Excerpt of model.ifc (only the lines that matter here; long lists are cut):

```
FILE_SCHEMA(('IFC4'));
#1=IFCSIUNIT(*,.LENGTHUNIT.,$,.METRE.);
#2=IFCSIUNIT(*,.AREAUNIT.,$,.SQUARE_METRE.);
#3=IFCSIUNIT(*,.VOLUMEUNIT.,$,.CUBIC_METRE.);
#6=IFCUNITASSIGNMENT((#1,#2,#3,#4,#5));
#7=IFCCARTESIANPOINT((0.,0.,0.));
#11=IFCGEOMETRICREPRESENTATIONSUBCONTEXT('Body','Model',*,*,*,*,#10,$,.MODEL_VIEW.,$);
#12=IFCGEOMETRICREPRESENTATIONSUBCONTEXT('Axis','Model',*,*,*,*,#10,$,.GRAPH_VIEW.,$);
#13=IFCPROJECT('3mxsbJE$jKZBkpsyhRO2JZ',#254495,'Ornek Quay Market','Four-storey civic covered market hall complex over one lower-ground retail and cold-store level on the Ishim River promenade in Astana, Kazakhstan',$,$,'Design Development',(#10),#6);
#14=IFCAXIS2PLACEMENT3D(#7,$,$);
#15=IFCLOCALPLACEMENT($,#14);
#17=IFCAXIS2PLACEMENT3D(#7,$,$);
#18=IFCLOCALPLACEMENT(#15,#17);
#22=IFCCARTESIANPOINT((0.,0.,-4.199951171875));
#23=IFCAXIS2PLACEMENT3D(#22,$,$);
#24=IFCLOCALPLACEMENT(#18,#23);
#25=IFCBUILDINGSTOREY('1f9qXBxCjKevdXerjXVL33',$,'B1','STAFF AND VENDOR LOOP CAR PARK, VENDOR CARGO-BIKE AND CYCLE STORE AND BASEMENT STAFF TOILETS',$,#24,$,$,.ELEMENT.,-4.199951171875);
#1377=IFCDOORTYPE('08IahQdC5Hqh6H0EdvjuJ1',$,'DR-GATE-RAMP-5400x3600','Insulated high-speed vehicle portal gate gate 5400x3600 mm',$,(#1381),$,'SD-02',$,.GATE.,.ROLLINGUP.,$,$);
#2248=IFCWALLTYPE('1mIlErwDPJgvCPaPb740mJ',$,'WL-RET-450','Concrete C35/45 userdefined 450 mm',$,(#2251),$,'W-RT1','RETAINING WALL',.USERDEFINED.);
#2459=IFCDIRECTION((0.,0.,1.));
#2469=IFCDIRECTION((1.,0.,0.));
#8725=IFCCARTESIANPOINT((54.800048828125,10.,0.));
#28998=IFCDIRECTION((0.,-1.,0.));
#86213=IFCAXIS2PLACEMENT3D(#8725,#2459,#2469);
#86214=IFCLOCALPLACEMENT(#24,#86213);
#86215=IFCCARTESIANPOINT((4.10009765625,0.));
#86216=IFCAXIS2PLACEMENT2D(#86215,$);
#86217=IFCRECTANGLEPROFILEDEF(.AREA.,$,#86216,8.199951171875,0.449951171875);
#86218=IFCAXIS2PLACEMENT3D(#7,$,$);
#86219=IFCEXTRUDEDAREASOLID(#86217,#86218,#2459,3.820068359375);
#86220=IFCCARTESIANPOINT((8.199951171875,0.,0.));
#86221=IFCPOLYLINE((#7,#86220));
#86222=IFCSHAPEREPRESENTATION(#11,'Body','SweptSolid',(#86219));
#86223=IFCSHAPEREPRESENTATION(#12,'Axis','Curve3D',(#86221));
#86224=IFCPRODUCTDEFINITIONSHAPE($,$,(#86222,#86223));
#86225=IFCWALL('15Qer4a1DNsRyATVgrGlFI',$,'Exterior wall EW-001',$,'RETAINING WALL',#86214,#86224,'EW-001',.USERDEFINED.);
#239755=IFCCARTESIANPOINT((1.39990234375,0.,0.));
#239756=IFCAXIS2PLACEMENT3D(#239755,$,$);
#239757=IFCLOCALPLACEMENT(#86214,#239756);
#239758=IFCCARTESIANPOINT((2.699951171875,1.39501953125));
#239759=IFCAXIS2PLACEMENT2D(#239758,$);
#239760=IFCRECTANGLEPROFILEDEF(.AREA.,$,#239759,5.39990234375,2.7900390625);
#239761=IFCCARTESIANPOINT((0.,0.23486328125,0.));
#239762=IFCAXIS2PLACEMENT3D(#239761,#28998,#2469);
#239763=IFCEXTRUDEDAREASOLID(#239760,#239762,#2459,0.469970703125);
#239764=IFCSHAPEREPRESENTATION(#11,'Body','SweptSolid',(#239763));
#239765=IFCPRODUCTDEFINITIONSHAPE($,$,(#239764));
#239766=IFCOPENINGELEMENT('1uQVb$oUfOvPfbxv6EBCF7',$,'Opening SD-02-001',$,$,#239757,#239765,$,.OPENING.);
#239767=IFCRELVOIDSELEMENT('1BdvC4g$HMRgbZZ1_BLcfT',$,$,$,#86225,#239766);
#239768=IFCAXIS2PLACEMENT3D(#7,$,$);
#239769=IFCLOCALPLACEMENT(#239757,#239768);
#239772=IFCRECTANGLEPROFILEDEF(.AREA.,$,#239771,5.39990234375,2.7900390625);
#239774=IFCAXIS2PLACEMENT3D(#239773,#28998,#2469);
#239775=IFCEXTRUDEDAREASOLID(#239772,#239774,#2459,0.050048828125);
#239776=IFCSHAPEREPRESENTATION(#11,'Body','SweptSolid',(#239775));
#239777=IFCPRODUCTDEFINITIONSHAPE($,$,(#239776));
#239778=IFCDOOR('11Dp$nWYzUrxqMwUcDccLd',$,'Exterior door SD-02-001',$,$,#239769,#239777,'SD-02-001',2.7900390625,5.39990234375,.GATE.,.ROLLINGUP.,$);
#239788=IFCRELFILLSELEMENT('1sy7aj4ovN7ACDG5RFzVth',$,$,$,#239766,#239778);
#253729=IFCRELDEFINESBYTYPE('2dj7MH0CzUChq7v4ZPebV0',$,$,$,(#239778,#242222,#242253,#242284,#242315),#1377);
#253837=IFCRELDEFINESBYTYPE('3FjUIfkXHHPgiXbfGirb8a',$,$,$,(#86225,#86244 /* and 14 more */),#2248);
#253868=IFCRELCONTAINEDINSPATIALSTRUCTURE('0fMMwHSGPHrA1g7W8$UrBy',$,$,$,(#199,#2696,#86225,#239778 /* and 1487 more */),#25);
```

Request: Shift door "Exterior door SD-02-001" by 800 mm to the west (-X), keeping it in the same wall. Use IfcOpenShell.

```python
import ifcopenshell
import ifcopenshell.api.geometry
import ifcopenshell.util.placement
import ifcopenshell.util.unit

model = ifcopenshell.open("model.ifc")
unit_scale = ifcopenshell.util.unit.calculate_unit_scale(model)

door = model.by_guid("11Dp$nWYzUrxqMwUcDccLd")
opening = door.FillsVoids[0].RelatingOpeningElement
wall = opening.VoidsElements[0].RelatingBuildingElement

wall_matrix = ifcopenshell.util.placement.get_local_placement(wall.ObjectPlacement)
shift = wall_matrix[:3, 0] * -0.8 / unit_scale
before = ifcopenshell.util.placement.get_local_placement(door.ObjectPlacement)[:3, 3].copy()

# The door is placed relative to its opening, so it follows when the opening moves.
matrix = ifcopenshell.util.placement.get_local_placement(opening.ObjectPlacement)
matrix[:3, 3] += shift
ifcopenshell.api.geometry.edit_object_placement(
    model, product=opening, matrix=matrix, is_si=False, should_transform_children=True
)

after = ifcopenshell.util.placement.get_local_placement(door.ObjectPlacement)[:3, 3]
print("door moved by", (after - before).round(3) + 0.0)

model.write("model_rev.ifc")
```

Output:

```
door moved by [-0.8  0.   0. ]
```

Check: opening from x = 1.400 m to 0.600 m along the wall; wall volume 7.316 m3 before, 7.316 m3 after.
